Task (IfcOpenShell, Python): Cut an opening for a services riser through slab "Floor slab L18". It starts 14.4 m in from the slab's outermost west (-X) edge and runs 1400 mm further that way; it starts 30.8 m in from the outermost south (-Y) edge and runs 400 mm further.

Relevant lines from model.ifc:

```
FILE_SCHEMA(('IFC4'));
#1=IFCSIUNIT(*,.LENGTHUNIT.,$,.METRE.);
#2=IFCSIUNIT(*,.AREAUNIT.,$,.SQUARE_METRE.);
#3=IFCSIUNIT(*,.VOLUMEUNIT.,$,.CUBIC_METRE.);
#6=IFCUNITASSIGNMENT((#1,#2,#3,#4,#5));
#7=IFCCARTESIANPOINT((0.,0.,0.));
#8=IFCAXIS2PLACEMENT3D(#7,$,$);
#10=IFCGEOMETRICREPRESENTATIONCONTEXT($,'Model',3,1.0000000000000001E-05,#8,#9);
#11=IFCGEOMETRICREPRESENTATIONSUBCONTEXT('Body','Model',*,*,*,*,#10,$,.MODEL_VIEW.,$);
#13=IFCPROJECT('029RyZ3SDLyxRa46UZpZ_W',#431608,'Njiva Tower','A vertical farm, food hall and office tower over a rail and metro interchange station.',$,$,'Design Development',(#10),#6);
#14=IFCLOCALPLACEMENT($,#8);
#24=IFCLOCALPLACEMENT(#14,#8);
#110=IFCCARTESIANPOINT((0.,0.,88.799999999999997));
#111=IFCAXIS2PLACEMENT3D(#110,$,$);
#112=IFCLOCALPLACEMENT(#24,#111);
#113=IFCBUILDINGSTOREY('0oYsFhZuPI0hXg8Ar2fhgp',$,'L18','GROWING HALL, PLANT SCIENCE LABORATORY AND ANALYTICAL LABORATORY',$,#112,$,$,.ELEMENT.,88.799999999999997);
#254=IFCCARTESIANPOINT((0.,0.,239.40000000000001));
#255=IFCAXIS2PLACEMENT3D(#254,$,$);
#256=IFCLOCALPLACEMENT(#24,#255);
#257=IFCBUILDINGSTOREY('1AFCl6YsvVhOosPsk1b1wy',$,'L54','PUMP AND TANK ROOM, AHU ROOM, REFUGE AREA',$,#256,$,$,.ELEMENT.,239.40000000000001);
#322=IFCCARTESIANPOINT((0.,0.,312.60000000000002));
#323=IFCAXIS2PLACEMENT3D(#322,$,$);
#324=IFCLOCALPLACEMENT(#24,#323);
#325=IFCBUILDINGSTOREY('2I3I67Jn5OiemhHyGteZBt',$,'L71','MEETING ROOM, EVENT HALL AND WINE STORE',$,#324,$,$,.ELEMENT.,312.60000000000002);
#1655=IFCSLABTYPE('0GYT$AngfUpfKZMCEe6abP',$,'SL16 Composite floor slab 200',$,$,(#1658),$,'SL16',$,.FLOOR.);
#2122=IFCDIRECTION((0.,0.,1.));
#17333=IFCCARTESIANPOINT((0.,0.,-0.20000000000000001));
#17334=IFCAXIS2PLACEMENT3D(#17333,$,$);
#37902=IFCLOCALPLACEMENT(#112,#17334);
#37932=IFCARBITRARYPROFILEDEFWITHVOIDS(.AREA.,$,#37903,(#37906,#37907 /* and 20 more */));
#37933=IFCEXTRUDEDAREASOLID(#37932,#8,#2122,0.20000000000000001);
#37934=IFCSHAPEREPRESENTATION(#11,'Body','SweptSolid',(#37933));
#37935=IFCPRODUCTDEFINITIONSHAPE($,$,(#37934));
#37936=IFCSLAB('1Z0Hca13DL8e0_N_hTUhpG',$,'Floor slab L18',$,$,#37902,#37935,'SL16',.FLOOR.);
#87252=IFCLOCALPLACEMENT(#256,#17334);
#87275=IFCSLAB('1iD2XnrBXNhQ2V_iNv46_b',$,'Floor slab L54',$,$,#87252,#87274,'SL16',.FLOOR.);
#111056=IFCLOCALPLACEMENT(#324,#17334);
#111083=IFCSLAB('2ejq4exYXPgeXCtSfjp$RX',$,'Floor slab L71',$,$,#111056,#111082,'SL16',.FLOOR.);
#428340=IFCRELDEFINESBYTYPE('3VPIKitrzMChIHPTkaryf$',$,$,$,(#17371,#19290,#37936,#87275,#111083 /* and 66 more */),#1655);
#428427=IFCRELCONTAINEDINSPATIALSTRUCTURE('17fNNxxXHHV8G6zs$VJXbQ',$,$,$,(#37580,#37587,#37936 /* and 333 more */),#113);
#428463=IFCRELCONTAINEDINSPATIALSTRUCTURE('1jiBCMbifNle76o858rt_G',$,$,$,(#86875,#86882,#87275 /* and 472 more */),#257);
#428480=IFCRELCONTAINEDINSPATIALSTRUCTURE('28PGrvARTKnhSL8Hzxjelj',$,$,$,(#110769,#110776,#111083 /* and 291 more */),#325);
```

```python
import numpy as np
import ifcopenshell
import ifcopenshell.api.feature
import ifcopenshell.api.geometry
import ifcopenshell.api.root
import ifcopenshell.geom
import ifcopenshell.util.placement
import ifcopenshell.util.representation
import ifcopenshell.util.shape
import ifcopenshell.util.unit

model = ifcopenshell.open("model.ifc")
unit_scale = ifcopenshell.util.unit.calculate_unit_scale(model)
settings = ifcopenshell.geom.settings()


def volume(element):
    """Net volume in cubic metres, openings subtracted."""
    shape = ifcopenshell.geom.create_shape(settings, element)
    return ifcopenshell.util.shape.get_volume(shape.geometry)


slab = model.by_id(37936)
before = volume(slab)

# Extent in the slab's own axes, in metres. The edges named are its -X and -Y sides.
slab_shape = ifcopenshell.geom.create_shape(settings, slab)
vertices = ifcopenshell.util.shape.get_vertices(slab_shape.geometry)
x_min, y_min, bottom = vertices.min(axis=0)
top = vertices[:, 2].max()

opening = ifcopenshell.api.root.create_entity(model, ifc_class="IfcOpeningElement", name="Services riser opening", predefined_type="OPENING")
context = ifcopenshell.util.representation.get_context(model, "Model", "Body", "MODEL_VIEW")
width, depth = 1.4, 0.4
outline = [(0.0, 0.0), (width, 0.0), (width, depth), (0.0, depth), (0.0, 0.0)]
# Overshoot both faces by 50 mm so the cut is clean.
shape = ifcopenshell.api.geometry.add_slab_representation(
    model, context=context, depth=top - bottom + 0.1, polyline=outline
)
ifcopenshell.api.geometry.assign_representation(model, product=opening, representation=shape)

matrix = ifcopenshell.util.placement.get_local_placement(slab.ObjectPlacement)
matrix[:, 3] = matrix @ np.append(np.array([x_min + 14.4, y_min + 30.8, bottom - 0.05]) / unit_scale, 1.0)
ifcopenshell.api.geometry.edit_object_placement(model, product=opening, matrix=matrix, is_si=False)
ifcopenshell.api.feature.add_feature(model, feature=opening, element=slab)

after = volume(slab)

print(f"slab volume {before:.3f} -> {after:.3f} m3")

model.write("model_rev.ifc")
```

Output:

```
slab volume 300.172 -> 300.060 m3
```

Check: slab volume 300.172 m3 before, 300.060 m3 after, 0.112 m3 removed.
